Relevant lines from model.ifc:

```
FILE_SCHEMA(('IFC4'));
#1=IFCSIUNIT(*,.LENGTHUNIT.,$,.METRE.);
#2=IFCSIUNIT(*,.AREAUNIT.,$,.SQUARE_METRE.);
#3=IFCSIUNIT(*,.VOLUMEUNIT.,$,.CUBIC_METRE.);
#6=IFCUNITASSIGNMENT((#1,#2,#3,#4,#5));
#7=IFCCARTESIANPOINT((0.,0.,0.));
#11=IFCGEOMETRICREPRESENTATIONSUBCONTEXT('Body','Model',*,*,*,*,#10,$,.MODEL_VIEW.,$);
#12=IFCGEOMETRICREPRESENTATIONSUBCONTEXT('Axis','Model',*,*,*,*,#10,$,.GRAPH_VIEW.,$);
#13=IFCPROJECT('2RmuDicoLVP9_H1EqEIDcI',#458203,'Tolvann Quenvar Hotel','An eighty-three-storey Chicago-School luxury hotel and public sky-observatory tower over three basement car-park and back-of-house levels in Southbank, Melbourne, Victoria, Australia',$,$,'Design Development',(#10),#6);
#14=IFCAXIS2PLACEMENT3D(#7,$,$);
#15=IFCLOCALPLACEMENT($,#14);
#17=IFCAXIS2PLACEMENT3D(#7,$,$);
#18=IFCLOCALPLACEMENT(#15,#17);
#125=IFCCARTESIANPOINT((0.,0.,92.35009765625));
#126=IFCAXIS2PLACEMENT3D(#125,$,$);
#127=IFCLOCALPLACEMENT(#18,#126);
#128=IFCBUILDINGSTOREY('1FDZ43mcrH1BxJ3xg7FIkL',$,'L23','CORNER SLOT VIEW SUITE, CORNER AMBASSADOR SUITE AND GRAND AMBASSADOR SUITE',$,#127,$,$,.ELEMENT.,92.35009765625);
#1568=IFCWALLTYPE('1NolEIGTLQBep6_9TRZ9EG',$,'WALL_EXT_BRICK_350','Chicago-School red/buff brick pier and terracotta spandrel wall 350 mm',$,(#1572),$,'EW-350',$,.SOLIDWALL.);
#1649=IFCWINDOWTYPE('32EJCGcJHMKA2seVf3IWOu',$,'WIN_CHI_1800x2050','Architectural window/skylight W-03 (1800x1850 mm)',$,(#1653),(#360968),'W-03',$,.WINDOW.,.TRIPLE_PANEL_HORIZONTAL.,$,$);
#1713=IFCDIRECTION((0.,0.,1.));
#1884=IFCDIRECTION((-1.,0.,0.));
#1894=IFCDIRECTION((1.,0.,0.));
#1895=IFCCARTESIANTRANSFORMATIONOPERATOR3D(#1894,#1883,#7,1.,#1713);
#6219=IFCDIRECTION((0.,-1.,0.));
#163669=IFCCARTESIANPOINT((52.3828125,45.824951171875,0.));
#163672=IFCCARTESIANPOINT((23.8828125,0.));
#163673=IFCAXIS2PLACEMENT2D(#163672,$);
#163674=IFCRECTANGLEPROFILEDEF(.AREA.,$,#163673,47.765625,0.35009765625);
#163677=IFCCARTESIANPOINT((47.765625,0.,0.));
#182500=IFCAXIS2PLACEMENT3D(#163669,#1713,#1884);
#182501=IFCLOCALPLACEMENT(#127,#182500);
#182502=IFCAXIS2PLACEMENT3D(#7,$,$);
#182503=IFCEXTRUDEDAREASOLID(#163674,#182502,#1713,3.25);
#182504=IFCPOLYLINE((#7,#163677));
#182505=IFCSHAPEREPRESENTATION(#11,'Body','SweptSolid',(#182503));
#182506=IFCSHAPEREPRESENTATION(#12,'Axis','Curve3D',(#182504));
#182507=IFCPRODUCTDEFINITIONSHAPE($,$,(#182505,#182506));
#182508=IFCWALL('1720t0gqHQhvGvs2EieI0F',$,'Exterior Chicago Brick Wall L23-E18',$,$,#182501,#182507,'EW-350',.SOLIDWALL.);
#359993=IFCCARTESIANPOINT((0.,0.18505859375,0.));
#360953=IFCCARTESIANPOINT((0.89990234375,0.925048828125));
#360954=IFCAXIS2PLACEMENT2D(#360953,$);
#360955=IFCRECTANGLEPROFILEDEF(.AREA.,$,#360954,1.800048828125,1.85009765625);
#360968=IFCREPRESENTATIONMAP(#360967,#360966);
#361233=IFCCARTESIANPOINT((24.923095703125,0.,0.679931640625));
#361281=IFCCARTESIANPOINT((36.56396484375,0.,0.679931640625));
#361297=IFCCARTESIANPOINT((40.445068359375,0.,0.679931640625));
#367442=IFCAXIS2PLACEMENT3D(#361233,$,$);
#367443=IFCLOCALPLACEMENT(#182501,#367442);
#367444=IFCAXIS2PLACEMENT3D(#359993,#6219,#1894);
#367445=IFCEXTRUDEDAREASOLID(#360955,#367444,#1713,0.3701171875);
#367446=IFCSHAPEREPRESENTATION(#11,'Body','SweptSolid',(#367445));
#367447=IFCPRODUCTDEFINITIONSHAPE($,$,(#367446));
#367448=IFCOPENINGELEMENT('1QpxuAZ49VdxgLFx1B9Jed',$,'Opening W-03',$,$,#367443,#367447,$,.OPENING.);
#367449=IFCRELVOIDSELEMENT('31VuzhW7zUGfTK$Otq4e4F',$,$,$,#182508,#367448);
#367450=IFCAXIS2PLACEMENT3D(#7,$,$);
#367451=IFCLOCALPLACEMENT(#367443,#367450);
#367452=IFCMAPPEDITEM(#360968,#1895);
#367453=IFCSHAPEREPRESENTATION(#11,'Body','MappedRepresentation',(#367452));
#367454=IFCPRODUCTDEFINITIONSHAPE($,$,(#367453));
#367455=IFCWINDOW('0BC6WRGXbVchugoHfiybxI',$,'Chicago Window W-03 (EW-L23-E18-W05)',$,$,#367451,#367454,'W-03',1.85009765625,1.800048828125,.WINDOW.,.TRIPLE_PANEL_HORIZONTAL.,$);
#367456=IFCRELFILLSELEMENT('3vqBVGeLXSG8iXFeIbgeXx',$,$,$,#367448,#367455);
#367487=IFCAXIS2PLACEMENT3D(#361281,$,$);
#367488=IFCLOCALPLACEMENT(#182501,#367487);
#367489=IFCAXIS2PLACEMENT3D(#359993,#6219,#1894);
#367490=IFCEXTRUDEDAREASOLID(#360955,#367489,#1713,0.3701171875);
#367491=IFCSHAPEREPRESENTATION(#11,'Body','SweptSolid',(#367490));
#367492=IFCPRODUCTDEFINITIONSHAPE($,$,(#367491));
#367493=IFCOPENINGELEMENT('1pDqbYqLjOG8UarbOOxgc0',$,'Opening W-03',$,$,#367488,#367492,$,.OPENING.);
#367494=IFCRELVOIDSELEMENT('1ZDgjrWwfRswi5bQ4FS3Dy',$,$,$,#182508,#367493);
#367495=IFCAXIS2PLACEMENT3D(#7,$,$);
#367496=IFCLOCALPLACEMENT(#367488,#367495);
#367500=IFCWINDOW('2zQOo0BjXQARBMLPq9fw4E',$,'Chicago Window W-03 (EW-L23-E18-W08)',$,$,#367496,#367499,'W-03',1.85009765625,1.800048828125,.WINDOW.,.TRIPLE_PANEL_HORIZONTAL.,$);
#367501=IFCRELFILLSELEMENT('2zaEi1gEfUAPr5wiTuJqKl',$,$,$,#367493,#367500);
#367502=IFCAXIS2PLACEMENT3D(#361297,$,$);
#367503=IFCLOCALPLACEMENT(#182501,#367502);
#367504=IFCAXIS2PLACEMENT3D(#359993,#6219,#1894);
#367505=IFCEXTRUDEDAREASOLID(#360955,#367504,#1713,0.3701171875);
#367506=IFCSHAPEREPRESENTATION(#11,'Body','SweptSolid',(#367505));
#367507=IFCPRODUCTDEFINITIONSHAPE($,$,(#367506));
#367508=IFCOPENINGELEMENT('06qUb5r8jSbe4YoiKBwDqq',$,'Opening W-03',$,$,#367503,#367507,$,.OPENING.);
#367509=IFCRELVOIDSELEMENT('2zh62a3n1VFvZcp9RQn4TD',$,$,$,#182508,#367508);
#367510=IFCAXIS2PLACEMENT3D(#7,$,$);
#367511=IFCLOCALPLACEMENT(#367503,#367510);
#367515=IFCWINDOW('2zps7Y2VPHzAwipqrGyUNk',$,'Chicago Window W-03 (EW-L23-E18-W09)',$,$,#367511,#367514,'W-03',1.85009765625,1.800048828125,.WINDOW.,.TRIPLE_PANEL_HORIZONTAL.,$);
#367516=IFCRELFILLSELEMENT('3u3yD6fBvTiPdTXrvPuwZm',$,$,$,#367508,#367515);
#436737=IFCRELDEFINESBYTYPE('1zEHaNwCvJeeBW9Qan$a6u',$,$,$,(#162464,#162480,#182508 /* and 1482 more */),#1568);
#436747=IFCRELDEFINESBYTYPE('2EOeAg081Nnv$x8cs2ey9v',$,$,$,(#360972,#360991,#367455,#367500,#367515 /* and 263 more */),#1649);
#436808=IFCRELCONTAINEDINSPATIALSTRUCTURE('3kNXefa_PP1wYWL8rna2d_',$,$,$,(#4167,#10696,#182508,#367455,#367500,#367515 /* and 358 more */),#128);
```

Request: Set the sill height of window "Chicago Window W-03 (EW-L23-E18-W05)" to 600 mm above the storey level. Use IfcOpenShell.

```python
import numpy as np
import ifcopenshell
import ifcopenshell.api.geometry
import ifcopenshell.geom
import ifcopenshell.util.element
import ifcopenshell.util.placement
import ifcopenshell.util.shape
import ifcopenshell.util.unit

model = ifcopenshell.open("model.ifc")
unit_scale = ifcopenshell.util.unit.calculate_unit_scale(model)

window = model.by_guid("0BC6WRGXbVchugoHfiybxI")
opening = window.FillsVoids[0].RelatingOpeningElement
storey = ifcopenshell.util.element.get_container(window, ifc_class="IfcBuildingStorey")
level = ifcopenshell.util.placement.get_local_placement(storey.ObjectPlacement)[2, 3]

# The opening's origin need not be at the sill, so measure its lowest point.
shape = ifcopenshell.geom.create_shape(ifcopenshell.geom.settings(), opening)
bottom = ifcopenshell.util.shape.get_shape_bottom_elevation(shape, shape.geometry) / unit_scale
dz = level + 0.6 / unit_scale - bottom

shift = np.array([0.0, 0.0, dz])
# The window is placed relative to its opening, so it follows when the opening moves.
matrix = ifcopenshell.util.placement.get_local_placement(opening.ObjectPlacement)
matrix[:3, 3] += shift
ifcopenshell.api.geometry.edit_object_placement(
    model, product=opening, matrix=matrix, is_si=False, should_transform_children=True
)

print(f"moved by {dz * unit_scale:+.3f} m")

model.write("model-out.ifc")
```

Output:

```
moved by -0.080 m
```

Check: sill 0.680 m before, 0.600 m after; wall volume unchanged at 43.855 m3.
